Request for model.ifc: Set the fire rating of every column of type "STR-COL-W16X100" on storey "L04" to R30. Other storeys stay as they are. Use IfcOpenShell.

First a look at what the model holds.

```python
import ifcopenshell
import ifcopenshell.util.element

model = ifcopenshell.open("model.ifc")
print(model.schema)
storey = next(s for s in model.by_type("IfcBuildingStorey") if s.Name == "L04")
columns = [e for e in ifcopenshell.util.element.get_decomposition(storey) if e.is_a("IfcColumn")]
seen = {}
for e in columns:
    element_type = ifcopenshell.util.element.get_type(e)
    key = (element_type.Name if element_type != e and element_type else None, ifcopenshell.util.element.get_pset(e, "Pset_ColumnCommon", "FireRating"))
    seen[key] = seen.get(key, 0) + 1
for (name, value), count in sorted(seen.items(), key=str):
    print(count, "x", name, "|", value)
```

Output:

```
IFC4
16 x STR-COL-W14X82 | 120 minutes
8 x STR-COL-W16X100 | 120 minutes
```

```python
import ifcopenshell
import ifcopenshell.api.pset
import ifcopenshell.util.element

model = ifcopenshell.open("model.ifc")

storey = next(s for s in model.by_type("IfcBuildingStorey") if s.Name == "L04")
columns = [e for e in ifcopenshell.util.element.get_decomposition(storey) if e.is_a("IfcColumn")]

count = 0
for e in columns:
    element_type = ifcopenshell.util.element.get_type(e)
    if element_type in (None, e) or element_type.Name != "STR-COL-W16X100":
        continue
    # add_pset returns the element's existing set when there is one.
    pset = ifcopenshell.api.pset.add_pset(model, product=e, name="Pset_ColumnCommon")
    ifcopenshell.api.pset.edit_pset(model, pset=pset, properties={"FireRating": "R30"})
    count += 1

print(count, "columns updated")

model.write("model_v2.ifc")
```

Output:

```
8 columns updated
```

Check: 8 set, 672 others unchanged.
